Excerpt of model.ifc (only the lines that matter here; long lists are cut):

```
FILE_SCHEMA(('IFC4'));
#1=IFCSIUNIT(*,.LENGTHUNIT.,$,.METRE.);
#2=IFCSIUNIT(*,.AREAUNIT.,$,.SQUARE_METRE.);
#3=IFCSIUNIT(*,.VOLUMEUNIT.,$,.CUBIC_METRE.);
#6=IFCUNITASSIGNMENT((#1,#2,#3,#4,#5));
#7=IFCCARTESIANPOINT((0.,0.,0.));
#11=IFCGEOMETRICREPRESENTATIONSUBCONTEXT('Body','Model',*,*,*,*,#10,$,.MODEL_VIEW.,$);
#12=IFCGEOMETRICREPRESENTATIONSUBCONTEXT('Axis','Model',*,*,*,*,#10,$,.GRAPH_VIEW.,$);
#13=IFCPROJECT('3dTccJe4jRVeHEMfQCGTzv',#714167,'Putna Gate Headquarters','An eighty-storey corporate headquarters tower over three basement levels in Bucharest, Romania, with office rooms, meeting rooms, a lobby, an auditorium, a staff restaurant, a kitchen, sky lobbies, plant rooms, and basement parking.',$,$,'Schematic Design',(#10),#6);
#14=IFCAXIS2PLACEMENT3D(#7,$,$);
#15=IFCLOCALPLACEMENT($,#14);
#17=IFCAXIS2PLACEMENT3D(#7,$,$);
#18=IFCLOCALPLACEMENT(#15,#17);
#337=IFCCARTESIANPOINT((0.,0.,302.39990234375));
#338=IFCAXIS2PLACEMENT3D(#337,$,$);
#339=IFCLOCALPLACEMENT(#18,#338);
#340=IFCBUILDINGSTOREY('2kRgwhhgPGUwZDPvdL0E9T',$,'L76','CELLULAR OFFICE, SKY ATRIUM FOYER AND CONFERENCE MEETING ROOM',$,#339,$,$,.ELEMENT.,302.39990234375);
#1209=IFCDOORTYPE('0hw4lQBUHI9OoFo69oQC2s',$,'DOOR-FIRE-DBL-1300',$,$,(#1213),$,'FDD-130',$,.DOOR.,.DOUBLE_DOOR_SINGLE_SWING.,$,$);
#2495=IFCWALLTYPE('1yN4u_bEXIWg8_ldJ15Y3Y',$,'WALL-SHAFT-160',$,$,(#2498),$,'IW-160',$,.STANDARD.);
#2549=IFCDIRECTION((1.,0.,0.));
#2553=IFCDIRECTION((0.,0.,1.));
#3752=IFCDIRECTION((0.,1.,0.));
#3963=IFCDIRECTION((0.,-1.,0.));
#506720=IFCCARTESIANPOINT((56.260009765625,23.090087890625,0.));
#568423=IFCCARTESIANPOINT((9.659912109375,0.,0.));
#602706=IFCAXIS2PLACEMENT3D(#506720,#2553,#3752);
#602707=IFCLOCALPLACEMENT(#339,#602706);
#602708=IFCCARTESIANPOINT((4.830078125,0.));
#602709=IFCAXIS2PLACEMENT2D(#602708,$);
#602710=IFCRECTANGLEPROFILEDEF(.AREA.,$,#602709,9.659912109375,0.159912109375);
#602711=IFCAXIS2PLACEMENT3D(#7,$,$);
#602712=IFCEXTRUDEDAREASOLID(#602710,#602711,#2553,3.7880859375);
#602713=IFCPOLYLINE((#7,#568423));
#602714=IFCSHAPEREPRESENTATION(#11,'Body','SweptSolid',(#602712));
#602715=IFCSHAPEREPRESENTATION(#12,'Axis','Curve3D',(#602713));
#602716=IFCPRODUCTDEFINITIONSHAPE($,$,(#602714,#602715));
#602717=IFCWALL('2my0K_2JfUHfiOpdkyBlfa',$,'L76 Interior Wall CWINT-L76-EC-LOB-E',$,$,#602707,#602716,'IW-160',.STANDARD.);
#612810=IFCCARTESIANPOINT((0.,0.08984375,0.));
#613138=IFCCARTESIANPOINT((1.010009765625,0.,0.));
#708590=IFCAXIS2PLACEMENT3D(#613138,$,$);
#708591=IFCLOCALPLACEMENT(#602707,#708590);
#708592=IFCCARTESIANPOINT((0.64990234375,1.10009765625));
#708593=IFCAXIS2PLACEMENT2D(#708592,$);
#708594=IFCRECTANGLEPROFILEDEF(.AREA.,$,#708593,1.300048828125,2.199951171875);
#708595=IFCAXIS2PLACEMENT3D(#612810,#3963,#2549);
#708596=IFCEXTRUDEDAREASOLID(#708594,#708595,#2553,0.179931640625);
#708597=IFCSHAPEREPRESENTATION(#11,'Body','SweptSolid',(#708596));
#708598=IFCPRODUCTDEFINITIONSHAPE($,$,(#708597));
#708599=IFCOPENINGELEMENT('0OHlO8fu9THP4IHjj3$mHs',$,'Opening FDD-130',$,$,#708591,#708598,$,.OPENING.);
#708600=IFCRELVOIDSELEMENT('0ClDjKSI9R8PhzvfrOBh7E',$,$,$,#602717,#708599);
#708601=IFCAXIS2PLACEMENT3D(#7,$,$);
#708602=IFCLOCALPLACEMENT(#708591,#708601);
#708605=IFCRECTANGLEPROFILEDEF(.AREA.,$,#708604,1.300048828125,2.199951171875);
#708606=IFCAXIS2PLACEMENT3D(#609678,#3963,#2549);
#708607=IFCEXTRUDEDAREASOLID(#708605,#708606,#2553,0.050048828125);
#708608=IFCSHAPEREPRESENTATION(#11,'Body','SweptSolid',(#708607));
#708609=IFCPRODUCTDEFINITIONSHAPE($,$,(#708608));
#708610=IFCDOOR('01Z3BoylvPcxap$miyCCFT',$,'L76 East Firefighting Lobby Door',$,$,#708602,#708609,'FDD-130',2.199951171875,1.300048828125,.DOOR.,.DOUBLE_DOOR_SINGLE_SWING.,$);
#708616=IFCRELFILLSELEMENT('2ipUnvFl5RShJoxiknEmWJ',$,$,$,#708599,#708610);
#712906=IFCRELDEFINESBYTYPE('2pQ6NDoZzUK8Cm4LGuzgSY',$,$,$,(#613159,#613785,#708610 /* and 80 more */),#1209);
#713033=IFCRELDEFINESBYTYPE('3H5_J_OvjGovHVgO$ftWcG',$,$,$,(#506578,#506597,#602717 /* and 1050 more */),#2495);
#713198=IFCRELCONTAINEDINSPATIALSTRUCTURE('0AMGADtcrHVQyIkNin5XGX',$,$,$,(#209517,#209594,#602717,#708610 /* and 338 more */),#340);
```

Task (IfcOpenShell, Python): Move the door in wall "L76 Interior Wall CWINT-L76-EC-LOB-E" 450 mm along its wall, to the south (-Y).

```python
import ifcopenshell
import ifcopenshell.api.geometry
import ifcopenshell.util.placement

model = ifcopenshell.open("model.ifc")

door = model.by_id(708610)
opening = door.FillsVoids[0].RelatingOpeningElement
wall = opening.VoidsElements[0].RelatingBuildingElement

wall_matrix = ifcopenshell.util.placement.get_local_placement(wall.ObjectPlacement)
shift = wall_matrix[:3, 0] * -0.45
before = ifcopenshell.util.placement.get_local_placement(door.ObjectPlacement)[:3, 3].copy()

# The door is placed relative to its opening, so it follows when the opening moves.
matrix = ifcopenshell.util.placement.get_local_placement(opening.ObjectPlacement)
matrix[:3, 3] += shift
ifcopenshell.api.geometry.edit_object_placement(
    model, product=opening, matrix=matrix, is_si=False, should_transform_children=True
)

after = ifcopenshell.util.placement.get_local_placement(door.ObjectPlacement)[:3, 3]
print("door moved by", (after - before).round(3) + 0.0)

model.write("model_v2.ifc")
```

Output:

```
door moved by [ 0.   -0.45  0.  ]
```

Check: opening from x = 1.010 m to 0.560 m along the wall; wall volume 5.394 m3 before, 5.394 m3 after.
